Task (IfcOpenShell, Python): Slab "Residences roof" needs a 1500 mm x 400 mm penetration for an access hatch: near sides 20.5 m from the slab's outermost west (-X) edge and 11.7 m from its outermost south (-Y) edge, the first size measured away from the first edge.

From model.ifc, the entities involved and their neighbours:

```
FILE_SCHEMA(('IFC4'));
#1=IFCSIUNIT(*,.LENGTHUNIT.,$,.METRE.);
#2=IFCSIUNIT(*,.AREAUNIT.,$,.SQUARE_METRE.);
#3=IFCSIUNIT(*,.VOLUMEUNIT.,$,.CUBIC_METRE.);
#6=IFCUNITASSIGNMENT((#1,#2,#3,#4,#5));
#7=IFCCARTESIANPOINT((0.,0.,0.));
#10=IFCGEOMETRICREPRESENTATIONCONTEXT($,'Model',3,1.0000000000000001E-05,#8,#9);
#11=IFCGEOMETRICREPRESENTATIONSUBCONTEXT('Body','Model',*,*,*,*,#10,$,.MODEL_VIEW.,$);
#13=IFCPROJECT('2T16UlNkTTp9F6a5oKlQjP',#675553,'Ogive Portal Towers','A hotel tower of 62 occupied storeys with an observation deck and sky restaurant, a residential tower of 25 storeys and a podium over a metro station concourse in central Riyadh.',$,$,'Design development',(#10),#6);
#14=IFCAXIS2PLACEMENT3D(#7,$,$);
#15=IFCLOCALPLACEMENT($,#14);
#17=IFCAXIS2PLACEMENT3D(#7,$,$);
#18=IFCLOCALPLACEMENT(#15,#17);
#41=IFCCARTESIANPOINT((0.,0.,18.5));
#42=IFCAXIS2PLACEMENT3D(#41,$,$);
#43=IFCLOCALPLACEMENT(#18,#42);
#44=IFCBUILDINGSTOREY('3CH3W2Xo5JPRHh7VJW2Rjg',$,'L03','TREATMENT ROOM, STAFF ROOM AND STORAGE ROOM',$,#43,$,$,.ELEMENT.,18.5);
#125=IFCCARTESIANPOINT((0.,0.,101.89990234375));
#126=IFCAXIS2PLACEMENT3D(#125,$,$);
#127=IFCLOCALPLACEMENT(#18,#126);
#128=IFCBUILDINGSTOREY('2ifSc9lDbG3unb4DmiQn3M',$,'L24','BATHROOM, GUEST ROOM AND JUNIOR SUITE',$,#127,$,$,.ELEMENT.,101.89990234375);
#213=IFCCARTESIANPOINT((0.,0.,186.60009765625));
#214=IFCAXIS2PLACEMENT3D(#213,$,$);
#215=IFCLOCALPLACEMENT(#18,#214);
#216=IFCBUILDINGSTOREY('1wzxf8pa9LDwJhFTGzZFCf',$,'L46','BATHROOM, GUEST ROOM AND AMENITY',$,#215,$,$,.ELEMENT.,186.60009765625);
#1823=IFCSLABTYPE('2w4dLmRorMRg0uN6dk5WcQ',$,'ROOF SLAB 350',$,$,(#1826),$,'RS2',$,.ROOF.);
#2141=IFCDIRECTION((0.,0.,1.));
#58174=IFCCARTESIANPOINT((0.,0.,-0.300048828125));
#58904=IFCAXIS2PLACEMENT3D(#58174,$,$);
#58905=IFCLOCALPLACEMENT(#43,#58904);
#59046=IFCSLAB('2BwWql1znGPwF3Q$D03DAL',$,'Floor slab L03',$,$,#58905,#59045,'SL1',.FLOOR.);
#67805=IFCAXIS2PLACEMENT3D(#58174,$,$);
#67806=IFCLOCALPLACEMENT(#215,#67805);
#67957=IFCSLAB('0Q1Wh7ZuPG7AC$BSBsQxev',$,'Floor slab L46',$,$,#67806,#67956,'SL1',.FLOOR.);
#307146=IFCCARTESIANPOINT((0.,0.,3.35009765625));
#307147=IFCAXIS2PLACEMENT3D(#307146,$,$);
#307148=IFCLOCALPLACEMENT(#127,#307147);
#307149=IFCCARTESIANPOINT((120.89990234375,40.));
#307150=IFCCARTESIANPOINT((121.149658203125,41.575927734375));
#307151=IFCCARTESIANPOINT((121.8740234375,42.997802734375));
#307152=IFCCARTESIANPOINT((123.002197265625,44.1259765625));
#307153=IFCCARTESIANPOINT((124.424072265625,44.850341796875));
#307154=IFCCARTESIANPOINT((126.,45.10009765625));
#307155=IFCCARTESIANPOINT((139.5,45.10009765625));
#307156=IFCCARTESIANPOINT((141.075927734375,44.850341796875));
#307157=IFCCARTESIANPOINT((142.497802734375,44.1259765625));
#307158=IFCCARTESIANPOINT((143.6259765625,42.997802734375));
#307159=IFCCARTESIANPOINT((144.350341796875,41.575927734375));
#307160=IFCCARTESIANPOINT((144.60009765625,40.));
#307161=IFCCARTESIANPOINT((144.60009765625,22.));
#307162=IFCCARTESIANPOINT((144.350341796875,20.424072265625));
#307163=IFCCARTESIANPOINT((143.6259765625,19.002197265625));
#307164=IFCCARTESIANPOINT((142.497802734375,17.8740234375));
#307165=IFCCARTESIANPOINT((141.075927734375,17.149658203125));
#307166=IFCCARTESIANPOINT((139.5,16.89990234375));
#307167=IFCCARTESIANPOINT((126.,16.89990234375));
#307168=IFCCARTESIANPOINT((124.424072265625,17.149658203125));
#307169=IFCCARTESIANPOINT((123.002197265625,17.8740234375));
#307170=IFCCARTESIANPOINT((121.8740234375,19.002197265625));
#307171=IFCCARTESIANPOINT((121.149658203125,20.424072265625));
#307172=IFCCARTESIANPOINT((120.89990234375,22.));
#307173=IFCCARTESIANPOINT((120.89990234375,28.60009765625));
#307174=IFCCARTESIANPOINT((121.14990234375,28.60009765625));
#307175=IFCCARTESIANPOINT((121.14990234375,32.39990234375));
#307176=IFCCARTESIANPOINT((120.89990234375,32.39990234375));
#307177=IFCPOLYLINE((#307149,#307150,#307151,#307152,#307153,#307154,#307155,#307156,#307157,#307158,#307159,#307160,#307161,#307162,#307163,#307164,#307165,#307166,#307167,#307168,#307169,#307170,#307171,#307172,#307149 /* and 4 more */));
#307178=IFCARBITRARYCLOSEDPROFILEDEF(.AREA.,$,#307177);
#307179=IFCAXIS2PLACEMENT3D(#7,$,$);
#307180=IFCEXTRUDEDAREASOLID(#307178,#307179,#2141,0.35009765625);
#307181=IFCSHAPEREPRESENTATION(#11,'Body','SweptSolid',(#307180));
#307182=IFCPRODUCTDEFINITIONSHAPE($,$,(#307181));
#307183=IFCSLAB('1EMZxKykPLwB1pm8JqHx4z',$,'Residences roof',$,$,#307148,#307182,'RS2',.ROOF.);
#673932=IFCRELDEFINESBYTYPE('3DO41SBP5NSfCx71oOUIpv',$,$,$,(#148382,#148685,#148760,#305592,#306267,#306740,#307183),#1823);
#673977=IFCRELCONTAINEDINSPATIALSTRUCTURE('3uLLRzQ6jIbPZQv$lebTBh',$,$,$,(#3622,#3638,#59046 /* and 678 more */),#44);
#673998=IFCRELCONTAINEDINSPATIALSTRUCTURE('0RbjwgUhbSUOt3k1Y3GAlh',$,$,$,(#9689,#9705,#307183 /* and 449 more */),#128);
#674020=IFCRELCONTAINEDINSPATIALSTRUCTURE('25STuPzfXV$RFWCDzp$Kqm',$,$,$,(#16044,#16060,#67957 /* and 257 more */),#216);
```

```python
import numpy as np
import ifcopenshell
import ifcopenshell.api.feature
import ifcopenshell.api.geometry
import ifcopenshell.api.root
import ifcopenshell.geom
import ifcopenshell.util.placement
import ifcopenshell.util.representation
import ifcopenshell.util.shape
import ifcopenshell.util.unit

model = ifcopenshell.open("model.ifc")
unit_scale = ifcopenshell.util.unit.calculate_unit_scale(model)
settings = ifcopenshell.geom.settings()


def volume(element):
    """Net volume in cubic metres, openings subtracted."""
    shape = ifcopenshell.geom.create_shape(settings, element)
    return ifcopenshell.util.shape.get_volume(shape.geometry)


slab = model.by_guid("1EMZxKykPLwB1pm8JqHx4z")
before = volume(slab)

# Extent in the slab's own axes, in metres. The edges named are its -X and -Y sides.
slab_shape = ifcopenshell.geom.create_shape(settings, slab)
vertices = ifcopenshell.util.shape.get_vertices(slab_shape.geometry)
x_min, y_min, bottom = vertices.min(axis=0)
top = vertices[:, 2].max()

opening = ifcopenshell.api.root.create_entity(model, ifc_class="IfcOpeningElement", name="Access hatch opening", predefined_type="OPENING")
context = ifcopenshell.util.representation.get_context(model, "Model", "Body", "MODEL_VIEW")
width, depth = 1.5, 0.4
outline = [(0.0, 0.0), (width, 0.0), (width, depth), (0.0, depth), (0.0, 0.0)]
# Overshoot both faces by 50 mm so the cut is clean.
shape = ifcopenshell.api.geometry.add_slab_representation(
    model, context=context, depth=top - bottom + 0.1, polyline=outline
)
ifcopenshell.api.geometry.assign_representation(model, product=opening, representation=shape)

matrix = ifcopenshell.util.placement.get_local_placement(slab.ObjectPlacement)
matrix[:, 3] = matrix @ np.append(np.array([x_min + 20.5, y_min + 11.7, bottom - 0.05]) / unit_scale, 1.0)
ifcopenshell.api.geometry.edit_object_placement(model, product=opening, matrix=matrix, is_si=False)
ifcopenshell.api.feature.add_feature(model, feature=opening, element=slab)

after = volume(slab)

print(f"slab volume {before:.3f} -> {after:.3f} m3")

model.write("model_updated.ifc")
```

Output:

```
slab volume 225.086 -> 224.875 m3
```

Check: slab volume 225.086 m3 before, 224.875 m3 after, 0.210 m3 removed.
